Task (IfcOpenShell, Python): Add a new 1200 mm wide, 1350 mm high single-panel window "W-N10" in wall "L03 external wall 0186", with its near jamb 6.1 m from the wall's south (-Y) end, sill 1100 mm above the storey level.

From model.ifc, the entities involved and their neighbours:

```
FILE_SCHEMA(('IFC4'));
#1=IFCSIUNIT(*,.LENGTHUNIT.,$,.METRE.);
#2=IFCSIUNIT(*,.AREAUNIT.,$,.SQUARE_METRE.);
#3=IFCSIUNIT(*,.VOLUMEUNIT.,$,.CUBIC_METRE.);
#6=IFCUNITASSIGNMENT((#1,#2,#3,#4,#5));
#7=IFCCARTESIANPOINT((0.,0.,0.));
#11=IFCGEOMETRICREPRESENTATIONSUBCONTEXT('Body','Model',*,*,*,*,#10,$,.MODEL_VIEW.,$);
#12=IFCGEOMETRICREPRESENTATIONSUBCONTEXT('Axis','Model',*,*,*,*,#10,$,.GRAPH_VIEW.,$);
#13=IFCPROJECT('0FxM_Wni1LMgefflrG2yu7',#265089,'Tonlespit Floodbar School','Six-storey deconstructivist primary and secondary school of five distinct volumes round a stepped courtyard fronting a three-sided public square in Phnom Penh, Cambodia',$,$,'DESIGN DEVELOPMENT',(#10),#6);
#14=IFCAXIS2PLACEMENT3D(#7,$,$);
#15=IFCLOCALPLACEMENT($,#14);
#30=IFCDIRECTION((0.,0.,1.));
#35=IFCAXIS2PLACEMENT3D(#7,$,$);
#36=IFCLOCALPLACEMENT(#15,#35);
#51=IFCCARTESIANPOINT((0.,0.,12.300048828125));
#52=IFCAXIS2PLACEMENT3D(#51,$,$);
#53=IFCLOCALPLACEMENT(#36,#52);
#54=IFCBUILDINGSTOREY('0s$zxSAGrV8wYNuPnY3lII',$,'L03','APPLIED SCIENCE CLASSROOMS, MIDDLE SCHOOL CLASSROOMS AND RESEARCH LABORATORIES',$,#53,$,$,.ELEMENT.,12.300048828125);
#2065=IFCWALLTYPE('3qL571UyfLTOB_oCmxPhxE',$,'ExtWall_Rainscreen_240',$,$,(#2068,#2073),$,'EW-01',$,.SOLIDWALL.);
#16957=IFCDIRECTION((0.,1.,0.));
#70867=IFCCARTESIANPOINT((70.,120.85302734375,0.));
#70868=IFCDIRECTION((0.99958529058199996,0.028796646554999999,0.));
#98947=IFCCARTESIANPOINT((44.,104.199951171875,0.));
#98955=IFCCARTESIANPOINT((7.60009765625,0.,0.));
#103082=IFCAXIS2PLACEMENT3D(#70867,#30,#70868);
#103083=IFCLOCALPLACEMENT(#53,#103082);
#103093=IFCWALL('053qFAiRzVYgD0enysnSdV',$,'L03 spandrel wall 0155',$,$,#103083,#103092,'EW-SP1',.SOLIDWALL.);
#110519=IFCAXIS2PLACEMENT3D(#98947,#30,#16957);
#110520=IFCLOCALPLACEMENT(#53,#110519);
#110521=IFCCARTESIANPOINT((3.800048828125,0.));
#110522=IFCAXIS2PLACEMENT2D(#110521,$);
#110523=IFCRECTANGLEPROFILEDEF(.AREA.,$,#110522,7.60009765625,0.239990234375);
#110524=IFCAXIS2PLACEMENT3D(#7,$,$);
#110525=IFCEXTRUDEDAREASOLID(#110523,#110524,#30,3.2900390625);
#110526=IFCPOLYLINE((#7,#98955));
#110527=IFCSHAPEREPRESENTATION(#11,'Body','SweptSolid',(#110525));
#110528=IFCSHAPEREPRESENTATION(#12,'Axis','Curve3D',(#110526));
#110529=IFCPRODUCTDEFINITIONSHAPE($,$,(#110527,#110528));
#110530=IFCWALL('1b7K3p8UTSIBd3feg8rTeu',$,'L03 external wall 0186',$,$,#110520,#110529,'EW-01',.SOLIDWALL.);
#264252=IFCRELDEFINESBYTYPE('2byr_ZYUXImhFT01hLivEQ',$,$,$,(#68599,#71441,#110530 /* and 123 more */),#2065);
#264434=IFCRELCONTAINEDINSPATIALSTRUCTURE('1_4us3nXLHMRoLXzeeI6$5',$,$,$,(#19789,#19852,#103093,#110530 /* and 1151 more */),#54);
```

```python
import numpy as np
import ifcopenshell
import ifcopenshell.api.feature
import ifcopenshell.api.geometry
import ifcopenshell.api.root
import ifcopenshell.api.spatial
import ifcopenshell.geom
import ifcopenshell.util.element
import ifcopenshell.util.placement
import ifcopenshell.util.representation
import ifcopenshell.util.shape
import ifcopenshell.util.unit

model = ifcopenshell.open("model.ifc")
unit_scale = ifcopenshell.util.unit.calculate_unit_scale(model)
settings = ifcopenshell.geom.settings()


def volume(element):
    """Net volume in cubic metres, openings subtracted."""
    shape = ifcopenshell.geom.create_shape(settings, element)
    return ifcopenshell.util.shape.get_volume(shape.geometry)


wall = model.by_id(110530)
storey = ifcopenshell.util.element.get_container(wall, ifc_class="IfcBuildingStorey")
context = ifcopenshell.util.representation.get_context(model, "Model", "Body", "MODEL_VIEW")
before = volume(wall)

width, height, from_end, sill = 1.2, 1.35, 6.1, 1.1  # metres

# The wall runs along its own X axis, and the end named is its -X end.
wall_shape = ifcopenshell.geom.create_shape(settings, wall)
x, y, z = ifcopenshell.util.shape.get_vertices(wall_shape.geometry).T
start = x.min() + from_end
face, thickness = float(y.min()), float(y.max() - y.min())
wall_matrix = ifcopenshell.util.placement.get_local_placement(wall.ObjectPlacement)
level = ifcopenshell.util.placement.get_local_placement(storey.ObjectPlacement)[2, 3]


def in_wall(x, y):
    """Placement at x, y metres in the wall's axes, at sill height."""
    matrix = wall_matrix.copy()
    matrix[:, 3] = wall_matrix @ np.array([x / unit_scale, y / unit_scale, 0.0, 1.0])
    matrix[2, 3] = level + sill / unit_scale
    return matrix


# Opening: a box that overshoots both wall faces by 50 mm.
opening = ifcopenshell.api.root.create_entity(model, ifc_class="IfcOpeningElement", predefined_type="OPENING")
box = ifcopenshell.api.geometry.add_wall_representation(
    model, context=context, length=width, height=height, thickness=thickness + 0.1
)
ifcopenshell.api.geometry.assign_representation(model, product=opening, representation=box)
ifcopenshell.api.geometry.edit_object_placement(model, product=opening, matrix=in_wall(start, face - 0.05), is_si=False)
ifcopenshell.api.feature.add_feature(model, feature=opening, element=wall)

window = ifcopenshell.api.root.create_entity(model, ifc_class="IfcWindow", name="W-N10", predefined_type="WINDOW")
window.OverallWidth, window.OverallHeight = width / unit_scale, height / unit_scale
window.PartitioningType = "SINGLE_PANEL"
body = ifcopenshell.api.geometry.add_window_representation(
    model,
    context=context,
    overall_width=window.OverallWidth,
    overall_height=window.OverallHeight,
    partition_type="SINGLE_PANEL",
)
ifcopenshell.api.geometry.assign_representation(model, product=window, representation=body)
ifcopenshell.api.spatial.assign_container(model, products=[window], relating_structure=storey)
ifcopenshell.api.feature.add_filling(model, opening=opening, element=window)

# Centre the window in the wall's thickness.
ifcopenshell.api.geometry.edit_object_placement(model, product=window, matrix=in_wall(start, face), is_si=False)
window_shape = ifcopenshell.geom.create_shape(settings, window)
depth = ifcopenshell.util.shape.get_vertices(window_shape.geometry)[:, 1]
offset = face + thickness / 2 - (depth.min() + depth.max()) / 2
ifcopenshell.api.geometry.edit_object_placement(model, product=window, matrix=in_wall(start, offset), is_si=False)

after = volume(wall)

print(f"wall volume {before:.3f} -> {after:.3f} m3")

model.write("model_updated.ifc")
```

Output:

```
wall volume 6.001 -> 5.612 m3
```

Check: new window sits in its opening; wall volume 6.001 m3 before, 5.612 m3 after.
